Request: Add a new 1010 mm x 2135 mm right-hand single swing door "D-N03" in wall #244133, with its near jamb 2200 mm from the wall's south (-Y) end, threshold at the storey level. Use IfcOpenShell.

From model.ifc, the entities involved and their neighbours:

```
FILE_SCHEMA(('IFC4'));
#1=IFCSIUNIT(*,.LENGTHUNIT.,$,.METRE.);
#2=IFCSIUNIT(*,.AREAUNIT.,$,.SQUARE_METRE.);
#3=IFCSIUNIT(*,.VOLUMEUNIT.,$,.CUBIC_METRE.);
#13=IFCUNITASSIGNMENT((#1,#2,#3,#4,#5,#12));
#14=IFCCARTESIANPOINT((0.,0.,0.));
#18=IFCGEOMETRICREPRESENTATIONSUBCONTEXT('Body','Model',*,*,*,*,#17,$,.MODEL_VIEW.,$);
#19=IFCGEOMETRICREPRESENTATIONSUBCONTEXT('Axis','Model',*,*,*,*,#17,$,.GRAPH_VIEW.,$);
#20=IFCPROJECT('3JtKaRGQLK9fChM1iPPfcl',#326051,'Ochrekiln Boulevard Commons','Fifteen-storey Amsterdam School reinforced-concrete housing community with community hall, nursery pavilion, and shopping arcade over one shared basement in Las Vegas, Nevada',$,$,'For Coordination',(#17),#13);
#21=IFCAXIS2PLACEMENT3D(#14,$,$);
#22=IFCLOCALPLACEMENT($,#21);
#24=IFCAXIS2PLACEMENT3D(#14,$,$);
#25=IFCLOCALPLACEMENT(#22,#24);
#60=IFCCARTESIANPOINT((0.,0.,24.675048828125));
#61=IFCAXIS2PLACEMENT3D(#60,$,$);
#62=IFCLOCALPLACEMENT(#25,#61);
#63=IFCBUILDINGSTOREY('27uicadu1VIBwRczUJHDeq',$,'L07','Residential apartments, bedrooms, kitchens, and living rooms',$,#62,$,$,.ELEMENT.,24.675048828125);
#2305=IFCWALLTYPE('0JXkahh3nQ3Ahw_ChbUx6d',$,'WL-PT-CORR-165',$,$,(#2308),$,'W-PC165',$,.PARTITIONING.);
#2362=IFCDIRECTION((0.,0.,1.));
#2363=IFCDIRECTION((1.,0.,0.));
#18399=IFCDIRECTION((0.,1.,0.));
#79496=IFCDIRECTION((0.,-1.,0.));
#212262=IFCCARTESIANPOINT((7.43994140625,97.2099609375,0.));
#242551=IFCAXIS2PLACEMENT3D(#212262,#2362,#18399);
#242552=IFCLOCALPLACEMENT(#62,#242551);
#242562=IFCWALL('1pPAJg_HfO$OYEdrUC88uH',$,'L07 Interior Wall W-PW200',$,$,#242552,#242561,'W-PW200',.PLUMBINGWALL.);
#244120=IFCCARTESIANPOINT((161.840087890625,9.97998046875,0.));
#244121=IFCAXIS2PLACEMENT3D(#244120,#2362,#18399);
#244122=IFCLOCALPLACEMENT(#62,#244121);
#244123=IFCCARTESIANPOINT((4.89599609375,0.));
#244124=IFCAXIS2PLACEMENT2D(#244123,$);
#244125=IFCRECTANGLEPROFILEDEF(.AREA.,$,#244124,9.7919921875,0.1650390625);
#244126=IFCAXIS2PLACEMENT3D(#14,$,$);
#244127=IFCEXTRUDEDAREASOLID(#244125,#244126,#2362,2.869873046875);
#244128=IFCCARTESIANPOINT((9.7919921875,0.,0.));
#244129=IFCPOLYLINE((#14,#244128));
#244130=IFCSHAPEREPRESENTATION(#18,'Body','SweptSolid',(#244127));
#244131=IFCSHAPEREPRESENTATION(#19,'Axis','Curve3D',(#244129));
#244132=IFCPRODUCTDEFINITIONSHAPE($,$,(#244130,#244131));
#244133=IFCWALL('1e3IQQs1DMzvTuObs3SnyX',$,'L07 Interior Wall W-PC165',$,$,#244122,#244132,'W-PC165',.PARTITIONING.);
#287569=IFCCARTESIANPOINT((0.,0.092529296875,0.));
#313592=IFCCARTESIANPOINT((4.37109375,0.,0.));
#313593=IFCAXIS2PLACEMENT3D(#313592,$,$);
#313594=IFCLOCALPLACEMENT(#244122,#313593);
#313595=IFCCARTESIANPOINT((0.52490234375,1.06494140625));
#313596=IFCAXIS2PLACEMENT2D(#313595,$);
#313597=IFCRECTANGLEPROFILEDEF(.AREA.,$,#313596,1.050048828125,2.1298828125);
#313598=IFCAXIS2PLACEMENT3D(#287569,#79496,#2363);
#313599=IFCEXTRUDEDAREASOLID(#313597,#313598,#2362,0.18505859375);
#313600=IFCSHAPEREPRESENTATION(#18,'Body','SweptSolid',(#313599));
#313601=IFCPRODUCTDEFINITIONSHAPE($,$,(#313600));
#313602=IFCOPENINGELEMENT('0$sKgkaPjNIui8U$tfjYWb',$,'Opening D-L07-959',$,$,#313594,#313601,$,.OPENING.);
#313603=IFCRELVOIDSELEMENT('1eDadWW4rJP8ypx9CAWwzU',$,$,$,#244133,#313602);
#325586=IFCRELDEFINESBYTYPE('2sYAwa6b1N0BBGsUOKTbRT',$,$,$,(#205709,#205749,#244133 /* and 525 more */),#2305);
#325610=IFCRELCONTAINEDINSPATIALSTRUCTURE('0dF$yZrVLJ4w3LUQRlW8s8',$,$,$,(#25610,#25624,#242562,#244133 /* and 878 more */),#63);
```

```python
import numpy as np
import ifcopenshell
import ifcopenshell.api.feature
import ifcopenshell.api.geometry
import ifcopenshell.api.root
import ifcopenshell.api.spatial
import ifcopenshell.geom
import ifcopenshell.util.element
import ifcopenshell.util.placement
import ifcopenshell.util.representation
import ifcopenshell.util.shape
import ifcopenshell.util.unit

model = ifcopenshell.open("model.ifc")
unit_scale = ifcopenshell.util.unit.calculate_unit_scale(model)
settings = ifcopenshell.geom.settings()


def volume(element):
    """Net volume in cubic metres, openings subtracted."""
    shape = ifcopenshell.geom.create_shape(settings, element)
    return ifcopenshell.util.shape.get_volume(shape.geometry)


wall = model.by_id(244133)
storey = ifcopenshell.util.element.get_container(wall, ifc_class="IfcBuildingStorey")
context = ifcopenshell.util.representation.get_context(model, "Model", "Body", "MODEL_VIEW")
before = volume(wall)

width, height, from_end, sill = 1.01, 2.135, 2.2, 0.0  # metres

# The wall runs along its own X axis, and the end named is its -X end.
wall_shape = ifcopenshell.geom.create_shape(settings, wall)
x, y, z = ifcopenshell.util.shape.get_vertices(wall_shape.geometry).T
start = x.min() + from_end
face, thickness = float(y.min()), float(y.max() - y.min())
wall_matrix = ifcopenshell.util.placement.get_local_placement(wall.ObjectPlacement)
level = ifcopenshell.util.placement.get_local_placement(storey.ObjectPlacement)[2, 3]


def in_wall(x, y):
    """Placement at x, y metres in the wall's axes, at sill height."""
    matrix = wall_matrix.copy()
    matrix[:, 3] = wall_matrix @ np.array([x / unit_scale, y / unit_scale, 0.0, 1.0])
    matrix[2, 3] = level + sill / unit_scale
    return matrix


# Opening: a box that overshoots both wall faces by 50 mm.
opening = ifcopenshell.api.root.create_entity(model, ifc_class="IfcOpeningElement", predefined_type="OPENING")
box = ifcopenshell.api.geometry.add_wall_representation(
    model, context=context, length=width, height=height, thickness=thickness + 0.1
)
ifcopenshell.api.geometry.assign_representation(model, product=opening, representation=box)
ifcopenshell.api.geometry.edit_object_placement(model, product=opening, matrix=in_wall(start, face - 0.05), is_si=False)
ifcopenshell.api.feature.add_feature(model, feature=opening, element=wall)

door = ifcopenshell.api.root.create_entity(model, ifc_class="IfcDoor", name="D-N03", predefined_type="DOOR")
door.OverallWidth, door.OverallHeight = width / unit_scale, height / unit_scale
door.OperationType = "SINGLE_SWING_RIGHT"
body = ifcopenshell.api.geometry.add_door_representation(
    model,
    context=context,
    overall_width=door.OverallWidth,
    overall_height=door.OverallHeight,
    operation_type="SINGLE_SWING_RIGHT",
    lining_properties={"LiningDepth": thickness / unit_scale, "ThresholdDepth": thickness / unit_scale},
)
ifcopenshell.api.geometry.assign_representation(model, product=door, representation=body)
ifcopenshell.api.spatial.assign_container(model, products=[door], relating_structure=storey)
ifcopenshell.api.feature.add_filling(model, opening=opening, element=door)

# The lining spans the wall, so the door starts at the wall face.
ifcopenshell.api.geometry.edit_object_placement(model, product=door, matrix=in_wall(start, face), is_si=False)

after = volume(wall)

print(f"wall volume {before:.3f} -> {after:.3f} m3")

model.write("model-out.ifc")
```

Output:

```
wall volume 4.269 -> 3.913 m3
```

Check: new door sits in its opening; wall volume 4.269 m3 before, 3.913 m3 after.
